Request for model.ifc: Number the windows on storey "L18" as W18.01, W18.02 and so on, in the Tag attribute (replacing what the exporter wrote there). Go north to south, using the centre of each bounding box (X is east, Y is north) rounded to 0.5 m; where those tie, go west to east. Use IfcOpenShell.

First a look at what the model holds.

```python
import ifcopenshell
import ifcopenshell.util.element
import ifcopenshell.util.placement

model = ifcopenshell.open("model.ifc")
print(model.schema)
storey = next(s for s in model.by_type("IfcBuildingStorey") if s.Name == "L18")
windows = [e for e in ifcopenshell.util.element.get_decomposition(storey) if e.is_a("IfcWindow")]
for e in sorted(windows, key=lambda e: e.id()):
    origin = ifcopenshell.util.placement.get_local_placement(e.ObjectPlacement)[:3, 3]
    print(e.id(), e.Tag, e.Name, origin.round(2) + 0.0, sep=" | ")
```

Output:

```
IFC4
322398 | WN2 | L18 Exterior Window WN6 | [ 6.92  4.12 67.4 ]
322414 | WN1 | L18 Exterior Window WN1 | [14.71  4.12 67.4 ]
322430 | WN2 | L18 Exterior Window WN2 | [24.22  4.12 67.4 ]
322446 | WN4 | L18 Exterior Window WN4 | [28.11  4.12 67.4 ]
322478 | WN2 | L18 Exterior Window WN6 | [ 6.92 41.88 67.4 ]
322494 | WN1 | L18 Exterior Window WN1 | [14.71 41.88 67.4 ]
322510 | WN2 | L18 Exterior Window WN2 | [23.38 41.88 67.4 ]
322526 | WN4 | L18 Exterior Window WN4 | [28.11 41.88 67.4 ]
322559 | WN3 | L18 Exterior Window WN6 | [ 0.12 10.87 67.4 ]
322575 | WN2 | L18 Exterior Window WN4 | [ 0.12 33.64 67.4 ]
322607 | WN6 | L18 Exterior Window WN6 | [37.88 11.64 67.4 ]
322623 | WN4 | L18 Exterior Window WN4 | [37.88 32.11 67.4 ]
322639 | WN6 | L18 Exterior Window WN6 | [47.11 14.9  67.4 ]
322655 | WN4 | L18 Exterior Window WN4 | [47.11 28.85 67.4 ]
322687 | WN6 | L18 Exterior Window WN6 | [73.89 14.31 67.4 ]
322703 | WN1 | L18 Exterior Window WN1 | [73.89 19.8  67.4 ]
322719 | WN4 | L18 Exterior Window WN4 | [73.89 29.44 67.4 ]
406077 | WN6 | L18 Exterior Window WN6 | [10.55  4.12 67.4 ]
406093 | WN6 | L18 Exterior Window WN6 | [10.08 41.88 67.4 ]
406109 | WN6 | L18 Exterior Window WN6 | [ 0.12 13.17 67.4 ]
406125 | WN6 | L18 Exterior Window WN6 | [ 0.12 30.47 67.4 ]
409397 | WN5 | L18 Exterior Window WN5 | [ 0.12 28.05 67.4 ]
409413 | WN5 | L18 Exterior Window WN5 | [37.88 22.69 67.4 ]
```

```python
import ifcopenshell
import ifcopenshell.geom
import ifcopenshell.util.element
import ifcopenshell.util.shape

model = ifcopenshell.open("model.ifc")
settings = ifcopenshell.geom.settings()
settings.set("use-world-coords", True)


def centre(element):
    shape = ifcopenshell.geom.create_shape(settings, element)
    return ifcopenshell.util.shape.get_bbox_centroid(shape.geometry)


storey = next(s for s in model.by_type("IfcBuildingStorey") if s.Name == "L18")
windows = [e for e in ifcopenshell.util.element.get_decomposition(storey) if e.is_a("IfcWindow")]

# Insertion points can sit at a corner or the storey origin, so sort by the geometry (in metres).
centres = {e: centre(e) for e in windows}
windows.sort(key=lambda e: (-round(centres[e][1] / 0.5), centres[e][0]))

for i, e in enumerate(windows, start=1):
    number = f"W18.{i:02d}"
    e.Tag = number
    print(e.id(), number)

model.write("model_v2.ifc")
```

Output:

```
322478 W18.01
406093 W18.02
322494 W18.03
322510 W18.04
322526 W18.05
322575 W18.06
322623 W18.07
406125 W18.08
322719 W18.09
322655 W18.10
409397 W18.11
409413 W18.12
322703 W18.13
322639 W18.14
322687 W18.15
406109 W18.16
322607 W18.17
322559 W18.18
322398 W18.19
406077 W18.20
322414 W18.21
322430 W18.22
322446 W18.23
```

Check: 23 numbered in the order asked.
